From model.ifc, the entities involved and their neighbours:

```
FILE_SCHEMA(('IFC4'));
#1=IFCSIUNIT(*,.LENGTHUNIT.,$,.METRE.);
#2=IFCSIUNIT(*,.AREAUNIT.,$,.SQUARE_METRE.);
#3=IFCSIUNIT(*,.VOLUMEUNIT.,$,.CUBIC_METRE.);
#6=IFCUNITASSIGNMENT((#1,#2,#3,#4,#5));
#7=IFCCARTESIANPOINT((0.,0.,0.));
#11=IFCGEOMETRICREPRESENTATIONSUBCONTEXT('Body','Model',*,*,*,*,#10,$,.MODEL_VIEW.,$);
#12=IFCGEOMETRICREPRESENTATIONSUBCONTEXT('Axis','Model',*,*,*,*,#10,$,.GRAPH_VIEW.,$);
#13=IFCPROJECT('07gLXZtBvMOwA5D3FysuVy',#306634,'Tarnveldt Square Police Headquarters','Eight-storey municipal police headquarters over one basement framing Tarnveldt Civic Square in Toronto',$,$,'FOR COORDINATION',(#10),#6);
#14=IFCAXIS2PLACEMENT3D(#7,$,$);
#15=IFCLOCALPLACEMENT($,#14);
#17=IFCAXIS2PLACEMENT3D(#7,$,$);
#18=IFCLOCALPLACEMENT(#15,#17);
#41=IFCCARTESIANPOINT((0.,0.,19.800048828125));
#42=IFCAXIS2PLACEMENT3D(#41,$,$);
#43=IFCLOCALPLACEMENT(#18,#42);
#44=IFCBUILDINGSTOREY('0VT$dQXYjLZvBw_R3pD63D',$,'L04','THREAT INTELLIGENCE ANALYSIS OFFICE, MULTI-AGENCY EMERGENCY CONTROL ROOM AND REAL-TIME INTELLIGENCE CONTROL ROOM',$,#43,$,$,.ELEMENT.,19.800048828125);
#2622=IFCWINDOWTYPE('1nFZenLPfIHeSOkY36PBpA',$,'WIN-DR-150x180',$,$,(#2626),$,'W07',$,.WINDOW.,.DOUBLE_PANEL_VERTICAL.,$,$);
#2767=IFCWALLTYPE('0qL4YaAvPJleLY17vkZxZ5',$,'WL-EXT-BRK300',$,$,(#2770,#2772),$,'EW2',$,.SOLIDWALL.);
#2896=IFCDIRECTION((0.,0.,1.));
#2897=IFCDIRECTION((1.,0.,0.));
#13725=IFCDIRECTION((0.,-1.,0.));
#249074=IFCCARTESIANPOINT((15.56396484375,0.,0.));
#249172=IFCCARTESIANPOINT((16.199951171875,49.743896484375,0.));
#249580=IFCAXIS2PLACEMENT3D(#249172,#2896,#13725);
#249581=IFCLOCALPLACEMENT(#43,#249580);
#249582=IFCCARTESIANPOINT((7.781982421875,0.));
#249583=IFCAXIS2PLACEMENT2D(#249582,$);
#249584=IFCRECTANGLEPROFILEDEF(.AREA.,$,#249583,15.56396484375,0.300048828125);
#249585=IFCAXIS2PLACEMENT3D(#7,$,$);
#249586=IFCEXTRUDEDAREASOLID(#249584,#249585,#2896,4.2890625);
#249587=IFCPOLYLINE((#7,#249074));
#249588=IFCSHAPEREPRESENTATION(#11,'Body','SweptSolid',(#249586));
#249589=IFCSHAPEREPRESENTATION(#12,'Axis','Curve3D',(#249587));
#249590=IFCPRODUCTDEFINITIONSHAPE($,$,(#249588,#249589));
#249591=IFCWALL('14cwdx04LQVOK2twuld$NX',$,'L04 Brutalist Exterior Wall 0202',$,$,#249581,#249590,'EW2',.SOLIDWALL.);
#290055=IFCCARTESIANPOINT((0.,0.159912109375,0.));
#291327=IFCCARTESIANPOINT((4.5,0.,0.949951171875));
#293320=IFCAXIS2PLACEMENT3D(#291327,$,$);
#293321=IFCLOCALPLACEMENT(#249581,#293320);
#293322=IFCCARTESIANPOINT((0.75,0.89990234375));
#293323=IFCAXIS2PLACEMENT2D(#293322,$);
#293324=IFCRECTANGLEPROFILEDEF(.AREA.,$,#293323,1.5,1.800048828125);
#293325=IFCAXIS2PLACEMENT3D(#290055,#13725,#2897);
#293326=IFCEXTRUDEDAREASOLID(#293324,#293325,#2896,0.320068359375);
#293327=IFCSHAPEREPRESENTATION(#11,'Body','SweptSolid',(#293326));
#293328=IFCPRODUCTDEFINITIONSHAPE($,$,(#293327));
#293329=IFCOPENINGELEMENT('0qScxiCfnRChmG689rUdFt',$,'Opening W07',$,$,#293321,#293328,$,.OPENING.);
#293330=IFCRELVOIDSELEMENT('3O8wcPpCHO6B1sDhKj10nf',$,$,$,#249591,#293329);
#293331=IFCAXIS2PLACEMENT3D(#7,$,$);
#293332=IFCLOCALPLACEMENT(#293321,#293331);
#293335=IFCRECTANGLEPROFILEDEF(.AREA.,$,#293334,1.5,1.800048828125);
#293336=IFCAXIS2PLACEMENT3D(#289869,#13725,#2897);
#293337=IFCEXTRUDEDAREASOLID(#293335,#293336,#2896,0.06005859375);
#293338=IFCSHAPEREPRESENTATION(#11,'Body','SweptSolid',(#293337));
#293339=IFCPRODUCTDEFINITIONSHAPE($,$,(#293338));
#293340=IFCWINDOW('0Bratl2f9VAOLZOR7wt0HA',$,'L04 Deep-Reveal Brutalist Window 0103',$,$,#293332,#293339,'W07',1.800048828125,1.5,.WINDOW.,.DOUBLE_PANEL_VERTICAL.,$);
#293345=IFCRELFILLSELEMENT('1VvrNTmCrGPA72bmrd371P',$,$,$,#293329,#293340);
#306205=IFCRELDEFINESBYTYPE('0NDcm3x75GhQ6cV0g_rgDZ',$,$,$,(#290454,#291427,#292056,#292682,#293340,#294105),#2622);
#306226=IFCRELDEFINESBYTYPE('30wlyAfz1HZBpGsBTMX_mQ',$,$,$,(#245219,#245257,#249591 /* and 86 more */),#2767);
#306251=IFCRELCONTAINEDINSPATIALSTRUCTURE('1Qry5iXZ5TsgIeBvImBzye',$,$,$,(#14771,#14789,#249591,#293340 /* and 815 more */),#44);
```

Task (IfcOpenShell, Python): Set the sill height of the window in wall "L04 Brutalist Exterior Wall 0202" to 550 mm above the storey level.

```python
import numpy as np
import ifcopenshell
import ifcopenshell.api.geometry
import ifcopenshell.geom
import ifcopenshell.util.element
import ifcopenshell.util.placement
import ifcopenshell.util.shape
import ifcopenshell.util.unit

model = ifcopenshell.open("model.ifc")
unit_scale = ifcopenshell.util.unit.calculate_unit_scale(model)

window = model.by_guid("0Bratl2f9VAOLZOR7wt0HA")
opening = window.FillsVoids[0].RelatingOpeningElement
storey = ifcopenshell.util.element.get_container(window, ifc_class="IfcBuildingStorey")
level = ifcopenshell.util.placement.get_local_placement(storey.ObjectPlacement)[2, 3]

# The opening's origin need not be at the sill, so measure its lowest point.
shape = ifcopenshell.geom.create_shape(ifcopenshell.geom.settings(), opening)
bottom = ifcopenshell.util.shape.get_shape_bottom_elevation(shape, shape.geometry) / unit_scale
dz = level + 0.55 / unit_scale - bottom

shift = np.array([0.0, 0.0, dz])
# The window is placed relative to its opening, so it follows when the opening moves.
matrix = ifcopenshell.util.placement.get_local_placement(opening.ObjectPlacement)
matrix[:3, 3] += shift
ifcopenshell.api.geometry.edit_object_placement(
    model, product=opening, matrix=matrix, is_si=False, should_transform_children=True
)

print(f"moved by {dz * unit_scale:+.3f} m")

model.write("model_updated.ifc")
```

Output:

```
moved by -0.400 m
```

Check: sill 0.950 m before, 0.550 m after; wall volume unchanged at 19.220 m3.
